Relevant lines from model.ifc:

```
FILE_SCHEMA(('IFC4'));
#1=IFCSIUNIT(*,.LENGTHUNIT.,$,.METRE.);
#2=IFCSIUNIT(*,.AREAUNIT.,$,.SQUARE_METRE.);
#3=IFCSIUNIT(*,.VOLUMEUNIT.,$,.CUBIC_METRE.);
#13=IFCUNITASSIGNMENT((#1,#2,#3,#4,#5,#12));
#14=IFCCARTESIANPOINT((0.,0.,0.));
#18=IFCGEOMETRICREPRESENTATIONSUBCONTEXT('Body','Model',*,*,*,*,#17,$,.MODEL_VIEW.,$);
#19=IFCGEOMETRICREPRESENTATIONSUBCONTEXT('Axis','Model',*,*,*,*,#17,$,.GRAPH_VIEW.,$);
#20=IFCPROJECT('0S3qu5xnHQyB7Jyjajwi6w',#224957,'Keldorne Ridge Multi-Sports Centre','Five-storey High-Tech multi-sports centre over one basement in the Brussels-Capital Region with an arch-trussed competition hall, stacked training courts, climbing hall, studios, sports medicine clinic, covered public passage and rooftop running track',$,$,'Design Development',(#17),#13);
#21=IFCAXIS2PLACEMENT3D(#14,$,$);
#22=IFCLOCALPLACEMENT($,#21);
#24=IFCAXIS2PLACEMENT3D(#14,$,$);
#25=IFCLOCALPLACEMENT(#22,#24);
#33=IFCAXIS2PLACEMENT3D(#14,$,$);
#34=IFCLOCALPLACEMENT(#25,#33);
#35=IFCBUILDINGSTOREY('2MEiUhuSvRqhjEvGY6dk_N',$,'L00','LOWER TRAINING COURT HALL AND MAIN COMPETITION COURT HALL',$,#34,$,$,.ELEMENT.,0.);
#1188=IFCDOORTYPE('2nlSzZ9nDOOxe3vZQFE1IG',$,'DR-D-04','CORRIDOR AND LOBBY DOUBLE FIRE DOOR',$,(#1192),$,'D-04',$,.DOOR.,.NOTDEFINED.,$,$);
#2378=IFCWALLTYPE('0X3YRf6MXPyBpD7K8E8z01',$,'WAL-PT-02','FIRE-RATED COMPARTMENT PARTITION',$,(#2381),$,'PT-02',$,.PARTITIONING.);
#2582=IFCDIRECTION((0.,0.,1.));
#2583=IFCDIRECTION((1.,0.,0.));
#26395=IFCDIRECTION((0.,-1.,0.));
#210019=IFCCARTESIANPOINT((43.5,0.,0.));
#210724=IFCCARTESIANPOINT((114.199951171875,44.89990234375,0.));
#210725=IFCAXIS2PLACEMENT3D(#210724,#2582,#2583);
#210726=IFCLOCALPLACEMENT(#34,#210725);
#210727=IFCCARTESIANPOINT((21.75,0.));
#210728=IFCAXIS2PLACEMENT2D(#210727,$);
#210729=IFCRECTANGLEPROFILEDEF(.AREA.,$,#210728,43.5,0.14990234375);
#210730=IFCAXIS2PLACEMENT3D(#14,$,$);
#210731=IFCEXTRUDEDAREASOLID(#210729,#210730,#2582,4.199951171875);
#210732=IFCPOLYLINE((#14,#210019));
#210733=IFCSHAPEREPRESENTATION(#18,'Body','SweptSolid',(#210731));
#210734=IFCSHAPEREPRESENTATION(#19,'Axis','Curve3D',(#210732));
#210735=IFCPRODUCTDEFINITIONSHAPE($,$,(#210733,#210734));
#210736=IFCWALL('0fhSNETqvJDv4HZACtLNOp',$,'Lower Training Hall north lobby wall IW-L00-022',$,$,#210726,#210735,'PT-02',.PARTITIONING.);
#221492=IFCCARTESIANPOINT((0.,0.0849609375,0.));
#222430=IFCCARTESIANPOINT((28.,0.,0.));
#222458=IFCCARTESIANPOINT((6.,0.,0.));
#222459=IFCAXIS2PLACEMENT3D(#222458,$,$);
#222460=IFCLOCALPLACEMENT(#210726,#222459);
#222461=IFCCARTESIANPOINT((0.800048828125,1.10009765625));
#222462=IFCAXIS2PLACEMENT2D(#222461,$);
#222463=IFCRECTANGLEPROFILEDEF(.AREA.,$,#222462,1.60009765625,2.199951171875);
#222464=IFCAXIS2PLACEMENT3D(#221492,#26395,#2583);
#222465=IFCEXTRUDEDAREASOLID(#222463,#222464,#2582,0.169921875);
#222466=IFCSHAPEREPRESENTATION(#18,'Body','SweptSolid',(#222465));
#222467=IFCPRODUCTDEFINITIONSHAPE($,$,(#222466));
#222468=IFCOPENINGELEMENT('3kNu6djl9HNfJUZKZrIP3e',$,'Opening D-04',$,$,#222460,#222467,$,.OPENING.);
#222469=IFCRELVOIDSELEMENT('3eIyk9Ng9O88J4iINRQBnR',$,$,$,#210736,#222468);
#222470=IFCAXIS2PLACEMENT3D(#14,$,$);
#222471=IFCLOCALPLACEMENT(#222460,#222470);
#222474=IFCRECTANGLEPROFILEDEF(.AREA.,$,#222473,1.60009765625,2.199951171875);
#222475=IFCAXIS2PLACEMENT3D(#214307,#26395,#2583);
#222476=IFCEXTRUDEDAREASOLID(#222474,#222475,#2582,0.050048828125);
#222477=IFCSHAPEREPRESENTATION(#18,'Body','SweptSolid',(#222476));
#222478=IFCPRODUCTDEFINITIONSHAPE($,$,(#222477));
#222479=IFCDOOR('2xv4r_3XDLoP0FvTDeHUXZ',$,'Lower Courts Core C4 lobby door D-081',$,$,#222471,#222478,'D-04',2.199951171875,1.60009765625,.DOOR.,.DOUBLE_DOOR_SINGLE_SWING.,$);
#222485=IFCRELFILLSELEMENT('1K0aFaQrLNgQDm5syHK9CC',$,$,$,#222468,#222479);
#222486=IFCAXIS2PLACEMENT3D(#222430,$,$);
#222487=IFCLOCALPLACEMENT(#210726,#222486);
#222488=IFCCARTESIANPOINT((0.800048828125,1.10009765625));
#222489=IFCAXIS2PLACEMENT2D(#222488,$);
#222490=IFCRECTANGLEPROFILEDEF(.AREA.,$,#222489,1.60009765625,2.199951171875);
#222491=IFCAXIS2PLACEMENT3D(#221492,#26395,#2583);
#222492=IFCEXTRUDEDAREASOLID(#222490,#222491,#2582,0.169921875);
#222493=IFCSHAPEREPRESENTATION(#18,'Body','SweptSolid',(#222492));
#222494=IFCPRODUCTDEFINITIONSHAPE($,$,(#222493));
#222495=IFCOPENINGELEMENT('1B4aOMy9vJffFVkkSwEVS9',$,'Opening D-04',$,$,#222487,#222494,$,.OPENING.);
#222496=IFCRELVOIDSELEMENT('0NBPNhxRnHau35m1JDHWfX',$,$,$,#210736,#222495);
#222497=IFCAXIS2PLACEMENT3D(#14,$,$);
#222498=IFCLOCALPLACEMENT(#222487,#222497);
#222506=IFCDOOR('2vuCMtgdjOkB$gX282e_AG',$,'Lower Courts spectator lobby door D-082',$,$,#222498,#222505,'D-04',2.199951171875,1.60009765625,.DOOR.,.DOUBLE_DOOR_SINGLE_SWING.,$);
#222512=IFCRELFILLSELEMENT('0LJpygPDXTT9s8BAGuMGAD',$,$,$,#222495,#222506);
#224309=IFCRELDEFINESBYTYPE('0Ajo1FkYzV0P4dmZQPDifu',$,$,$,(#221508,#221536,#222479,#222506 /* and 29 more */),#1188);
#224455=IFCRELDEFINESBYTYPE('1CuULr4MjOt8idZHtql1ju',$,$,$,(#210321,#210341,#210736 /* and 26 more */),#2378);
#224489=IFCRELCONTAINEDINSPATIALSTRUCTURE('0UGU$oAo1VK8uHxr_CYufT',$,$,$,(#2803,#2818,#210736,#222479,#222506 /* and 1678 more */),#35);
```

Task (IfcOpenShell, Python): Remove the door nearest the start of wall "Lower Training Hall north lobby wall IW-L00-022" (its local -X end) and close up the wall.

```python
import ifcopenshell
import ifcopenshell.api.feature
import ifcopenshell.api.root
import ifcopenshell.geom
import ifcopenshell.util.shape

model = ifcopenshell.open("model.ifc")
settings = ifcopenshell.geom.settings()


def volume(element):
    """Net volume in cubic metres, openings subtracted."""
    shape = ifcopenshell.geom.create_shape(settings, element)
    return ifcopenshell.util.shape.get_volume(shape.geometry)


door = model.by_guid("2xv4r_3XDLoP0FvTDeHUXZ")
opening = door.FillsVoids[0].RelatingOpeningElement
wall = opening.VoidsElements[0].RelatingBuildingElement
before = volume(wall)

ifcopenshell.api.root.remove_product(model, product=door)
ifcopenshell.api.feature.remove_feature(model, feature=opening)

after = volume(wall)

print(f"wall volume {before:.3f} -> {after:.3f} m3")

model.write("model_v2.ifc")
```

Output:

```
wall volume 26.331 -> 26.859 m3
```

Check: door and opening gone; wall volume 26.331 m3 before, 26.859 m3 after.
